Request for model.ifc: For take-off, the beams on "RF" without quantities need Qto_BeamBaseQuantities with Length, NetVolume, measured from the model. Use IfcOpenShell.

First a look at what the model holds.

```python
import ifcopenshell
import ifcopenshell.util.element
import ifcopenshell.util.unit

model = ifcopenshell.open("model.ifc")
print(model.schema)
for unit_type in ("LENGTHUNIT", "AREAUNIT", "VOLUMEUNIT"):
    print(unit_type, ifcopenshell.util.unit.calculate_unit_scale(model, unit_type))
storey = next(s for s in model.by_type("IfcBuildingStorey") if s.Name == "RF")
beams = [e for e in ifcopenshell.util.element.get_decomposition(storey) if e.is_a("IfcBeam")]
for e in sorted(beams, key=lambda e: e.id()):
    print(e.id(), e.is_a(), e.Name, list(ifcopenshell.util.element.get_psets(e, qtos_only=True)), sep=" | ")
```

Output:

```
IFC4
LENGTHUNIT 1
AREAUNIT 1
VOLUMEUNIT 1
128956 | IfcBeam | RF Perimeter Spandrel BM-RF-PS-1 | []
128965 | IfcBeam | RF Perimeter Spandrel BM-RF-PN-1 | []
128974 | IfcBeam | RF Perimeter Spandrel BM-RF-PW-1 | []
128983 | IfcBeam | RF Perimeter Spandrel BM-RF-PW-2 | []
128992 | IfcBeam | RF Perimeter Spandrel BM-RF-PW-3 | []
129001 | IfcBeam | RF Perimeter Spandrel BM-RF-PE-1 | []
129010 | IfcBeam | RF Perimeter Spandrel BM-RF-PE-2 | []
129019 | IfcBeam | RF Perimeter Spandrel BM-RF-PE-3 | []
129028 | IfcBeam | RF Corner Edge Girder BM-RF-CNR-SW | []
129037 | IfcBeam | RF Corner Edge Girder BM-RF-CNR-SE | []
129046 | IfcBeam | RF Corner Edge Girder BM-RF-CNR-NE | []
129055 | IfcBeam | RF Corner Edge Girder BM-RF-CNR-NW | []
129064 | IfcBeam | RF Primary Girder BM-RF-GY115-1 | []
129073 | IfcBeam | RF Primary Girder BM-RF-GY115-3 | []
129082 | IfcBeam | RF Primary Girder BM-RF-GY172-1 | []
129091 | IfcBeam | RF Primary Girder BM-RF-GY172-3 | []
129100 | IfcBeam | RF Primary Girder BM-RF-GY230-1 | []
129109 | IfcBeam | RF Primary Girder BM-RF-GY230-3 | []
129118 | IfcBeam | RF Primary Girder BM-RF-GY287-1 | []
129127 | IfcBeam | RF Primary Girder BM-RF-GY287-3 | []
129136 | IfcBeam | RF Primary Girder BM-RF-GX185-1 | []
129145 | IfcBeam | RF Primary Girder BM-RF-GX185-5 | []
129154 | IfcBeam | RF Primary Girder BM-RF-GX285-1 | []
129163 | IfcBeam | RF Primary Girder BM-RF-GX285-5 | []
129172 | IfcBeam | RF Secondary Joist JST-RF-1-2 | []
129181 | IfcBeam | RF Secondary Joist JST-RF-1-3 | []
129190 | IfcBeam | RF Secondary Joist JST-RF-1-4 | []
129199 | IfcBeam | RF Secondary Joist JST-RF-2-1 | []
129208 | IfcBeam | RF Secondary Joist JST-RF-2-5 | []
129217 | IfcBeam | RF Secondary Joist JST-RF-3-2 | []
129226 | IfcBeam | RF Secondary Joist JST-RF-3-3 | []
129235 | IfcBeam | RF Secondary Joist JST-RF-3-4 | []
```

```python
import ifcopenshell
import ifcopenshell.api.pset
import ifcopenshell.geom
import ifcopenshell.util.element
import ifcopenshell.util.shape
import ifcopenshell.util.unit

model = ifcopenshell.open("model.ifc")
unit_scale = ifcopenshell.util.unit.calculate_unit_scale(model)
volume_scale = ifcopenshell.util.unit.calculate_unit_scale(model, "VOLUMEUNIT")
settings = ifcopenshell.geom.settings()

storey = next(s for s in model.by_type("IfcBuildingStorey") if s.Name == "RF")
beams = [e for e in ifcopenshell.util.element.get_decomposition(storey) if e.is_a("IfcBeam")]

for e in sorted(beams, key=lambda e: e.id()):
    if ifcopenshell.util.element.get_psets(e, qtos_only=True, should_inherit=False):
        continue
    # Geometry comes back in metres, in the element's own axes.
    shape = ifcopenshell.geom.create_shape(settings, e)
    values = {
        "Length": ifcopenshell.util.shape.get_max_xyz(shape.geometry) / unit_scale,
        "NetVolume": ifcopenshell.util.shape.get_volume(shape.geometry) / volume_scale,
    }
    qto = ifcopenshell.api.pset.add_qto(model, product=e, name="Qto_BeamBaseQuantities")
    ifcopenshell.api.pset.edit_qto(model, qto=qto, properties=values)
    print(e.id(), {k: round(v, 3) for k, v in values.items()})

model.write("model-out.ifc")
```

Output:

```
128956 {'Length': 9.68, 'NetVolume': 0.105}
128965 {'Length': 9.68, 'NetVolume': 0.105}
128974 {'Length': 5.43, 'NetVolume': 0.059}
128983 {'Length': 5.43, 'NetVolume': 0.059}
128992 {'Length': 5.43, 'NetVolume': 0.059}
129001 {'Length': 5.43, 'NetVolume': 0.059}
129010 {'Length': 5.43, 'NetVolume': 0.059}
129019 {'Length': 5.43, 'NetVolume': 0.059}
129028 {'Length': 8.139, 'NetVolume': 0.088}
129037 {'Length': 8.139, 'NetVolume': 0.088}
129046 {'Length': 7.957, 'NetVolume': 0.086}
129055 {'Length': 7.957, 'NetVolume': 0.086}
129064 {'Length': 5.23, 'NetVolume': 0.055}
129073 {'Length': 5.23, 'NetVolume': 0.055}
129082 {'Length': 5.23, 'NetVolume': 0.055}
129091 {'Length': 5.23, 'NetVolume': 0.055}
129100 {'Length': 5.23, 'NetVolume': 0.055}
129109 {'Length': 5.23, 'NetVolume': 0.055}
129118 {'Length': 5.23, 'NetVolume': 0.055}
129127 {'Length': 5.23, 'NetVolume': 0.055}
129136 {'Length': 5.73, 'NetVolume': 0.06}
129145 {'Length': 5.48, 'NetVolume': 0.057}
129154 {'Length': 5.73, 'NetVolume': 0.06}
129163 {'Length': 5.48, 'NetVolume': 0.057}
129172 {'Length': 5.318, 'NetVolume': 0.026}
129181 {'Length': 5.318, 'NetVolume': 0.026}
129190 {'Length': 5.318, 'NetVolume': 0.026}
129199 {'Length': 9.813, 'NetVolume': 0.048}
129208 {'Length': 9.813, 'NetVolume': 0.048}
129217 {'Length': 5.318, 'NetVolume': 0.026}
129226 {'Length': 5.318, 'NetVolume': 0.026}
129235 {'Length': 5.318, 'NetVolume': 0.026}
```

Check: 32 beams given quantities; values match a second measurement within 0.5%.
